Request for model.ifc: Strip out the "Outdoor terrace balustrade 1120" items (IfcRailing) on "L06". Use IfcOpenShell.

First a look at what the model holds.

```python
import ifcopenshell
import ifcopenshell.util.element

model = ifcopenshell.open("model.ifc")
print(model.schema)
storey = next(s for s in model.by_type("IfcBuildingStorey") if s.Name == "L06")
railings = [e for e in ifcopenshell.util.element.get_decomposition(storey) if e.is_a("IfcRailing")]
seen = {}
for e in railings:
    element_type = ifcopenshell.util.element.get_type(e)
    name = element_type.Name if element_type not in (None, e) else None
    seen[name] = seen.get(name, 0) + 1
for name, count in sorted(seen.items(), key=str):
    print(count, "x", name)
```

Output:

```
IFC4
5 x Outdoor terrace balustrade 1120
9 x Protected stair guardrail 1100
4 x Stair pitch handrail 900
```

```python
import ifcopenshell
import ifcopenshell.api.root
import ifcopenshell.util.element

model = ifcopenshell.open("model.ifc")

storey = next(s for s in model.by_type("IfcBuildingStorey") if s.Name == "L06")
railings = [e for e in ifcopenshell.util.element.get_decomposition(storey) if e.is_a("IfcRailing")]
targets = [e for e in railings if (t := ifcopenshell.util.element.get_type(e)) not in (None, e) and t.Name == "Outdoor terrace balustrade 1120"]

for e in targets:
    ifcopenshell.api.root.remove_product(model, product=e)
print(len(targets), "removed")

model.write("model_v2.ifc")
```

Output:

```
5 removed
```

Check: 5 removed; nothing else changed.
